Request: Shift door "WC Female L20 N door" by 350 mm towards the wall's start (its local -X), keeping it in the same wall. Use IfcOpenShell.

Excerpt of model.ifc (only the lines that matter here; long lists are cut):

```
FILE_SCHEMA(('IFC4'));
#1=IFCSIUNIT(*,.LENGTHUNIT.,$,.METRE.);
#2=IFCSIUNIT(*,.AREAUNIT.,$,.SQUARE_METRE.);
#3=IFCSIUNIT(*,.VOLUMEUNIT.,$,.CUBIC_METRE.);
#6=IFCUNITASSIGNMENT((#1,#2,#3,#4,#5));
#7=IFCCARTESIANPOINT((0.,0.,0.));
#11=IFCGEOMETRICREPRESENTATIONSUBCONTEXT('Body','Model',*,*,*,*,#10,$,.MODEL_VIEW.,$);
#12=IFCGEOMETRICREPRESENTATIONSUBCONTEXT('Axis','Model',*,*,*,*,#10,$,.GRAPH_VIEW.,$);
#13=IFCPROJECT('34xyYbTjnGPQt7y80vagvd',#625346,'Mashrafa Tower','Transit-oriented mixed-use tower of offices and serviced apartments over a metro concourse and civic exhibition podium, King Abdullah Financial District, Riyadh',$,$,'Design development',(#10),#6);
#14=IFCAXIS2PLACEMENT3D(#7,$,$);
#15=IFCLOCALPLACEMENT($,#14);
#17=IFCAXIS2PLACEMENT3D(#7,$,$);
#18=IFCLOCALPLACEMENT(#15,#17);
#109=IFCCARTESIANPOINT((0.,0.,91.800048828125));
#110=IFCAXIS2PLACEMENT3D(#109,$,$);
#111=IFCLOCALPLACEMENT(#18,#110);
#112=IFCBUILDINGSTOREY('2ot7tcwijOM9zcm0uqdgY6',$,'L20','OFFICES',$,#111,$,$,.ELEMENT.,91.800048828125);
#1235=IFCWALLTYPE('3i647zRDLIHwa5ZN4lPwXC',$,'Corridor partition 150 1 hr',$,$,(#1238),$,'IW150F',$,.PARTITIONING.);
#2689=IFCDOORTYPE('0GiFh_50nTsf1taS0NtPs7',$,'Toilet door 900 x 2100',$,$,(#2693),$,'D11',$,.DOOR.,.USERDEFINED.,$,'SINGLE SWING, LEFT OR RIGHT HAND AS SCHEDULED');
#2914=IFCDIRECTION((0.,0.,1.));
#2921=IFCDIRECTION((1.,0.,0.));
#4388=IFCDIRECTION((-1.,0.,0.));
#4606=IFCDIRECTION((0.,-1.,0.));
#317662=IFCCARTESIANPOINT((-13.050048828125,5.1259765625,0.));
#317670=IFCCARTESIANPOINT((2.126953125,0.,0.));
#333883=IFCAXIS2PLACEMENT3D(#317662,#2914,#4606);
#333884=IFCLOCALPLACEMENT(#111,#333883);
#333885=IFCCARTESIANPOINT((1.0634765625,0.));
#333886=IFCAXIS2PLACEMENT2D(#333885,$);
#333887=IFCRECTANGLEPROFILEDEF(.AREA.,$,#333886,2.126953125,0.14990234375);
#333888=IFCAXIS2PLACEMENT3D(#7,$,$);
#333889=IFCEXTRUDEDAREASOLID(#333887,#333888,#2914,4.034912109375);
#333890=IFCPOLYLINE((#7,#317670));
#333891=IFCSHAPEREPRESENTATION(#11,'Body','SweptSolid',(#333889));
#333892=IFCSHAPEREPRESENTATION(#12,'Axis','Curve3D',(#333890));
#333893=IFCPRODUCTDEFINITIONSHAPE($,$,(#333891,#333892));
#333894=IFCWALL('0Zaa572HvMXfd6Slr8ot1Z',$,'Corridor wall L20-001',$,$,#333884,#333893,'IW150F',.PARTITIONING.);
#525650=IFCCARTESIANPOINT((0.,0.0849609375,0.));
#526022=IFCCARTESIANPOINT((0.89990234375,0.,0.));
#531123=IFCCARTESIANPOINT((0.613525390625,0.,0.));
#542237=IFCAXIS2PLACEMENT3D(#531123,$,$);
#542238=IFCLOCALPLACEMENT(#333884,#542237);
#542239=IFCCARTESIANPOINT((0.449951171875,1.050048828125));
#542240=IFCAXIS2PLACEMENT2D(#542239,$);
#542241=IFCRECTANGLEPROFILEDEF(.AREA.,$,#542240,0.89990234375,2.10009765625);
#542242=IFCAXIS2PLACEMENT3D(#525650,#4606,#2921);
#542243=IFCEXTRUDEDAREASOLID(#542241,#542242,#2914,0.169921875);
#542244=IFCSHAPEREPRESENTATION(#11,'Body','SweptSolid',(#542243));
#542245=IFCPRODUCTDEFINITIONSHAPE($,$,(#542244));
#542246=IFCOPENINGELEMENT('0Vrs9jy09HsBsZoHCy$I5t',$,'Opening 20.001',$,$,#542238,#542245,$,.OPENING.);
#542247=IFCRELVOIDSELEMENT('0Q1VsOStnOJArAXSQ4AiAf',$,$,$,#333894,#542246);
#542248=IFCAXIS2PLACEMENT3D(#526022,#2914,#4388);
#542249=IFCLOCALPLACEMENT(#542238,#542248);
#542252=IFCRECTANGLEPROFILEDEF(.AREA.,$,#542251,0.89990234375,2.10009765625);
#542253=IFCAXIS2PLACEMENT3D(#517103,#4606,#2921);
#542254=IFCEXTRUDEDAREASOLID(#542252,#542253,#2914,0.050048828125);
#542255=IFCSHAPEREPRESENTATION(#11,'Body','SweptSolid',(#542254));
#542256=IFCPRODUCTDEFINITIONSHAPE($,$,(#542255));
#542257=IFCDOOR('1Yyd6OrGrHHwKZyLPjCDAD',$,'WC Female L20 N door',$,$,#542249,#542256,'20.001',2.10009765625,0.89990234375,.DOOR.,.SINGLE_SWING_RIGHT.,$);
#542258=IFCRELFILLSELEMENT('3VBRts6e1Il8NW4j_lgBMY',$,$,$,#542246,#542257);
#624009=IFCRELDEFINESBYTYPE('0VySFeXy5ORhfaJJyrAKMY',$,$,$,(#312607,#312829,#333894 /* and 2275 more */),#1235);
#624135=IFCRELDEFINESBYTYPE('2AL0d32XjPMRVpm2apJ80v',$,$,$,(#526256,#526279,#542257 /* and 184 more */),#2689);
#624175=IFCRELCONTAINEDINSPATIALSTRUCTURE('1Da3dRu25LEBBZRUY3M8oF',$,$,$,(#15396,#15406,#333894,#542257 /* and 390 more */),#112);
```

```python
import ifcopenshell
import ifcopenshell.api.geometry
import ifcopenshell.util.placement
import ifcopenshell.util.unit

model = ifcopenshell.open("model.ifc")
unit_scale = ifcopenshell.util.unit.calculate_unit_scale(model)

door = model.by_guid("1Yyd6OrGrHHwKZyLPjCDAD")
opening = door.FillsVoids[0].RelatingOpeningElement
wall = opening.VoidsElements[0].RelatingBuildingElement

wall_matrix = ifcopenshell.util.placement.get_local_placement(wall.ObjectPlacement)
shift = wall_matrix[:3, 0] * -0.35 / unit_scale
before = ifcopenshell.util.placement.get_local_placement(door.ObjectPlacement)[:3, 3].copy()

# The door is placed relative to its opening, so it follows when the opening moves.
matrix = ifcopenshell.util.placement.get_local_placement(opening.ObjectPlacement)
matrix[:3, 3] += shift
ifcopenshell.api.geometry.edit_object_placement(
    model, product=opening, matrix=matrix, is_si=False, should_transform_children=True
)

after = ifcopenshell.util.placement.get_local_placement(door.ObjectPlacement)[:3, 3]
print("door moved by", (after - before).round(3) + 0.0)

model.write("model_v2.ifc")
```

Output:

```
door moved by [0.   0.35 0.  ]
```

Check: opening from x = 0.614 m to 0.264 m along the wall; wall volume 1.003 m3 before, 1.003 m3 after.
